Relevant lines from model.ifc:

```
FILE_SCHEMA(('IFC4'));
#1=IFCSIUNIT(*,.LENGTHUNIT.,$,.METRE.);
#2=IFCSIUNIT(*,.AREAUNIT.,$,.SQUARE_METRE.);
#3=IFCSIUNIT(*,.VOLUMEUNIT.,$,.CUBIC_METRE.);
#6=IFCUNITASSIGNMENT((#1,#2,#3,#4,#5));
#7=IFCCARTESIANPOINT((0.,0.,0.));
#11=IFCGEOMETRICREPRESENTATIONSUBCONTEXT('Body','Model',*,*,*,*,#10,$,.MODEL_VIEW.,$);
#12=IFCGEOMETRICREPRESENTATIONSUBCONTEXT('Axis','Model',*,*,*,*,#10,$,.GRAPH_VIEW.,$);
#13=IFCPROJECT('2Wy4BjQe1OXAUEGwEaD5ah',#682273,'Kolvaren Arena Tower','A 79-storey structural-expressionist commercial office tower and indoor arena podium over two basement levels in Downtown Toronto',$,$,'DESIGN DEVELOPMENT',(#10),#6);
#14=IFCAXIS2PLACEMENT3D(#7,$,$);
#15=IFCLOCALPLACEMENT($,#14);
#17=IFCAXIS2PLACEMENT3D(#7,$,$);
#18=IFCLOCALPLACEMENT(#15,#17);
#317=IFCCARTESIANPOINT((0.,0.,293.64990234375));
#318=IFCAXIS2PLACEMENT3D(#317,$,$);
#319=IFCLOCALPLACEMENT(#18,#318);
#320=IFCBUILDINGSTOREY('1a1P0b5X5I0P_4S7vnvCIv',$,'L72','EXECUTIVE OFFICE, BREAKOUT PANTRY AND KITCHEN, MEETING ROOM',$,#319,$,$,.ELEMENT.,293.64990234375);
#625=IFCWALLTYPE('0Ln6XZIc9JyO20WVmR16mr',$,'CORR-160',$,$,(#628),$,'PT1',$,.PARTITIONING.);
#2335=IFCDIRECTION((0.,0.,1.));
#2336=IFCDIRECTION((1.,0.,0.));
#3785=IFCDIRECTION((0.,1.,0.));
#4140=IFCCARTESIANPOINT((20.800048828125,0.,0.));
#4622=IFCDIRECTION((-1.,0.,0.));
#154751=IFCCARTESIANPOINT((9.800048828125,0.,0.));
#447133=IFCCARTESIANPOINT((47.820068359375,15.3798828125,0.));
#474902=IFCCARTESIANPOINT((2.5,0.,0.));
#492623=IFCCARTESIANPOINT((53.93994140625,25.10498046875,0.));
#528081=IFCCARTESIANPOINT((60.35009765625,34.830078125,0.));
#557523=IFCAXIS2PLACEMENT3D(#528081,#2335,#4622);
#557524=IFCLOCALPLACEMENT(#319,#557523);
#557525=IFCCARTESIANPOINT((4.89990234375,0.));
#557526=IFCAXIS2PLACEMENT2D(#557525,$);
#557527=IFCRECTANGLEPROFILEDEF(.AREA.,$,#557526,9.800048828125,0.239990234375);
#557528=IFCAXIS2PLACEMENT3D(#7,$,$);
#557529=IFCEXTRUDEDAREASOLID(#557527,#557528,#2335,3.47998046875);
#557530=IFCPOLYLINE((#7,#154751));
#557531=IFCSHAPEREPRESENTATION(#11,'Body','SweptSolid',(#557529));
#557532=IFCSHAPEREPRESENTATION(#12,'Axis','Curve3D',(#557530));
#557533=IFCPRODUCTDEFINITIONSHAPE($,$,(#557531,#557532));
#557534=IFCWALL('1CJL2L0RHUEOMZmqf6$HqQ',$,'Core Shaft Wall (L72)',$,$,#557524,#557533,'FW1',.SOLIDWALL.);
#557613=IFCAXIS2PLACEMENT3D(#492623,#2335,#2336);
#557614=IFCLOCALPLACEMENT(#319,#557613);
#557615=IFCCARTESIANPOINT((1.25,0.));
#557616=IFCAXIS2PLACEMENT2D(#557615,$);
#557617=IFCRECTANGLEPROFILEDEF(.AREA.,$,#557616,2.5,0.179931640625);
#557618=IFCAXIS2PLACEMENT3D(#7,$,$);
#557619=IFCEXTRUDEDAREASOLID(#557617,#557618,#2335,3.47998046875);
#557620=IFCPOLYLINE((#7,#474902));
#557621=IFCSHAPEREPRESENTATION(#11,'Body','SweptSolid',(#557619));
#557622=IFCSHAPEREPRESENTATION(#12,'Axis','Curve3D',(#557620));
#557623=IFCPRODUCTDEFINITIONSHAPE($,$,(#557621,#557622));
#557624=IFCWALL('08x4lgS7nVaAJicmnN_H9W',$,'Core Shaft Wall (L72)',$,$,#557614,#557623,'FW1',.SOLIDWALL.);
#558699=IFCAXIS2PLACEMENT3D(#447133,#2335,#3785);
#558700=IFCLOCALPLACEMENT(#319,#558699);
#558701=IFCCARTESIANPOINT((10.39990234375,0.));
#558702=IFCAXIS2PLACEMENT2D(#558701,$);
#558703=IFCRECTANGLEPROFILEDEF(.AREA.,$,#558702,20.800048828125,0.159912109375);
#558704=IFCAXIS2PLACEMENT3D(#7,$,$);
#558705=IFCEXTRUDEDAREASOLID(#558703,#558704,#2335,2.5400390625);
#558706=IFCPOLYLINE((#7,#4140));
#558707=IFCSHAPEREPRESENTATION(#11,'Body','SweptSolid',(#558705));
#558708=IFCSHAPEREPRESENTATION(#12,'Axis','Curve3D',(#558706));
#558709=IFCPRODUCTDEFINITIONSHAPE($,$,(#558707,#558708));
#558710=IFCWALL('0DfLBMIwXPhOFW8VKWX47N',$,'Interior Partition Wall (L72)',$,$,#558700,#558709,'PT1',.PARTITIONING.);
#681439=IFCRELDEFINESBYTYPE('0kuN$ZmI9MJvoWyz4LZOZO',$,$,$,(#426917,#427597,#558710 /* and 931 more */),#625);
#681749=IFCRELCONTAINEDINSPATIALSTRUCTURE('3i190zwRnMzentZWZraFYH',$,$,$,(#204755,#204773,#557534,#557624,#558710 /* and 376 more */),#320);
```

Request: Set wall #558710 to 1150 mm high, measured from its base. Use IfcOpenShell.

```python
import ifcopenshell
import ifcopenshell.geom
import ifcopenshell.util.representation
import ifcopenshell.util.shape
import ifcopenshell.util.unit

model = ifcopenshell.open("model.ifc")
unit_scale = ifcopenshell.util.unit.calculate_unit_scale(model)
settings = ifcopenshell.geom.settings()


def volume(element):
    """Net volume in cubic metres, openings subtracted."""
    shape = ifcopenshell.geom.create_shape(settings, element)
    return ifcopenshell.util.shape.get_volume(shape.geometry)


wall = model.by_guid("0DfLBMIwXPhOFW8VKWX47N")
before = volume(wall)

body = ifcopenshell.util.representation.get_representation(wall, "Model", "Body")
solid = body.Items[0]
old_height = solid.Depth
solid.Depth = 1.15 / unit_scale
after = volume(wall)

print(f"height {old_height:g} -> {solid.Depth:g}, volume {before:.3f} -> {after:.3f} m3")

model.write("model-out.ifc")
```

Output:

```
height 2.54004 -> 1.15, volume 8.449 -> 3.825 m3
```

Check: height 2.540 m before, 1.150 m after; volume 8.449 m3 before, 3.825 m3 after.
